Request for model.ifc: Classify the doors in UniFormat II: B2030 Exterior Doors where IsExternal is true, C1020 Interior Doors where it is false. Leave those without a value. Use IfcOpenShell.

First a look at what the model holds.

```python
import ifcopenshell
import ifcopenshell.util.element

model = ifcopenshell.open("model.ifc")
print(model.schema)
print("classifications:", [c.Name for c in model.by_type("IfcClassification")])
values = [ifcopenshell.util.element.get_pset(e, "Pset_DoorCommon", "IsExternal") for e in model.by_type("IfcDoor")]
for value in (True, False, None):
    print("IsExternal", value, values.count(value))
```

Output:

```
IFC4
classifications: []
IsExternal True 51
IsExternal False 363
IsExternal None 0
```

```python
import ifcopenshell
import ifcopenshell.api.classification
import ifcopenshell.util.element

model = ifcopenshell.open("model.ifc")

system = ifcopenshell.api.classification.add_classification(model, classification="UniFormat II")

doors = model.by_type("IfcDoor")
external = {e: ifcopenshell.util.element.get_pset(e, "Pset_DoorCommon", "IsExternal") for e in doors}
for flag, code, name in ((True, "B2030", "Exterior Doors"), (False, "C1020", "Interior Doors")):
    products = [e for e in doors if external[e] is flag]
    ifcopenshell.api.classification.add_reference(
        model, products=products, classification=system, identification=code, name=name
    )
    print(code, len(products))

model.write("model_rev.ifc")
```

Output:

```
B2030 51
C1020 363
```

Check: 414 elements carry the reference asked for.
